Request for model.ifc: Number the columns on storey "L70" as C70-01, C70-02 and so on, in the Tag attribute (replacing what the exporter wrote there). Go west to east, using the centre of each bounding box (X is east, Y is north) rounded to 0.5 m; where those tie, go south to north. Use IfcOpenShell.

First a look at what the model holds.

```python
import ifcopenshell
import ifcopenshell.util.element
import ifcopenshell.util.placement

model = ifcopenshell.open("model.ifc")
print(model.schema)
storey = next(s for s in model.by_type("IfcBuildingStorey") if s.Name == "L70")
columns = [e for e in ifcopenshell.util.element.get_decomposition(storey) if e.is_a("IfcColumn")]
for e in sorted(columns, key=lambda e: e.id()):
    origin = ifcopenshell.util.placement.get_local_placement(e.ObjectPlacement)[:3, 3]
    print(e.id(), e.Tag, e.Name, origin.round(2) + 0.0, sep=" | ")
```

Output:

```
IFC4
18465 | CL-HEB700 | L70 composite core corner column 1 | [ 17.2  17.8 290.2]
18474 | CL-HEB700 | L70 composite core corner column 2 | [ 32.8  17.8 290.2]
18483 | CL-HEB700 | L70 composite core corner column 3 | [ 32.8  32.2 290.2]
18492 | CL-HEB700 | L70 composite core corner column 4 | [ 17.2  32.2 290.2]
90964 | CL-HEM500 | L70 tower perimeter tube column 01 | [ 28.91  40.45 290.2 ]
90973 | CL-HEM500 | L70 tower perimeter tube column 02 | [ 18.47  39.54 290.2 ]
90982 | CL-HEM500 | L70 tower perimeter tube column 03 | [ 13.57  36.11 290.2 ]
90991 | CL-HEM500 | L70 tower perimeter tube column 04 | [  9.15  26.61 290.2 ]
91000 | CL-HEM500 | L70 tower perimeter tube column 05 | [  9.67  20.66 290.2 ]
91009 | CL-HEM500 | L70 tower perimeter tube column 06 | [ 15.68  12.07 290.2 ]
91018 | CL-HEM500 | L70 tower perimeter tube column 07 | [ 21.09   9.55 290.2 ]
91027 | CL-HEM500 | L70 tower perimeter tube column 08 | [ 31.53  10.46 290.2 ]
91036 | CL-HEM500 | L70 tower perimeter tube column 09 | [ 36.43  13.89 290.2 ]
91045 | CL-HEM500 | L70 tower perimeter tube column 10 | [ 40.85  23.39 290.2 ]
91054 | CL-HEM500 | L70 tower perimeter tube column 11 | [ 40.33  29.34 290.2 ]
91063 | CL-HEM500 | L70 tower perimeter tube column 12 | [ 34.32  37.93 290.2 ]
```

```python
import ifcopenshell
import ifcopenshell.geom
import ifcopenshell.util.element
import ifcopenshell.util.shape

model = ifcopenshell.open("model.ifc")
settings = ifcopenshell.geom.settings()
settings.set("use-world-coords", True)


def centre(element):
    shape = ifcopenshell.geom.create_shape(settings, element)
    return ifcopenshell.util.shape.get_bbox_centroid(shape.geometry)


storey = next(s for s in model.by_type("IfcBuildingStorey") if s.Name == "L70")
columns = [e for e in ifcopenshell.util.element.get_decomposition(storey) if e.is_a("IfcColumn")]

# Insertion points can sit at a corner or the storey origin, so sort by the geometry (in metres).
centres = {e: centre(e) for e in columns}
columns.sort(key=lambda e: (round(centres[e][0] / 0.5), centres[e][1]))

for i, e in enumerate(columns, start=1):
    number = f"C70-{i:02d}"
    e.Tag = number
    print(e.id(), number)

model.write("model_v2.ifc")
```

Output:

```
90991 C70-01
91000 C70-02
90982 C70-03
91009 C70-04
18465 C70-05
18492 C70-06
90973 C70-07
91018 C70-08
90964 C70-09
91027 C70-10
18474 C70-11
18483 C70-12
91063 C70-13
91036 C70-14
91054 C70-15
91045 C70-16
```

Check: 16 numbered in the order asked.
